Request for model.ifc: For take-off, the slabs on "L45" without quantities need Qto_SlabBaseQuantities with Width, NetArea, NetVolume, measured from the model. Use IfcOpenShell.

First a look at what the model holds.

```python
import ifcopenshell
import ifcopenshell.util.element
import ifcopenshell.util.unit

model = ifcopenshell.open("model.ifc")
print(model.schema)
for unit_type in ("LENGTHUNIT", "AREAUNIT", "VOLUMEUNIT"):
    print(unit_type, ifcopenshell.util.unit.calculate_unit_scale(model, unit_type))
storey = next(s for s in model.by_type("IfcBuildingStorey") if s.Name == "L45")
slabs = [e for e in ifcopenshell.util.element.get_decomposition(storey) if e.is_a("IfcSlab")]
for e in sorted(slabs, key=lambda e: e.id()):
    print(e.id(), e.is_a(), e.Name, list(ifcopenshell.util.element.get_psets(e, qtos_only=True)), sep=" | ")
```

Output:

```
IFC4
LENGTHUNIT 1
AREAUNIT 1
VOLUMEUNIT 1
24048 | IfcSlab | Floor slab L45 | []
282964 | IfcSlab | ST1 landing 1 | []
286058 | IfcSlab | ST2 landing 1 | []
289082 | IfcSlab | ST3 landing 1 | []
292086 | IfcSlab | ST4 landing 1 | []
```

```python
import ifcopenshell
import ifcopenshell.api.pset
import ifcopenshell.geom
import ifcopenshell.util.element
import ifcopenshell.util.shape
import ifcopenshell.util.unit

model = ifcopenshell.open("model.ifc")
unit_scale = ifcopenshell.util.unit.calculate_unit_scale(model)
area_scale = ifcopenshell.util.unit.calculate_unit_scale(model, "AREAUNIT")
volume_scale = ifcopenshell.util.unit.calculate_unit_scale(model, "VOLUMEUNIT")
settings = ifcopenshell.geom.settings()

storey = next(s for s in model.by_type("IfcBuildingStorey") if s.Name == "L45")
slabs = [e for e in ifcopenshell.util.element.get_decomposition(storey) if e.is_a("IfcSlab")]

for e in sorted(slabs, key=lambda e: e.id()):
    if ifcopenshell.util.element.get_psets(e, qtos_only=True, should_inherit=False):
        continue
    # Geometry comes back in metres, in the element's own axes.
    shape = ifcopenshell.geom.create_shape(settings, e)
    values = {
        "Width": ifcopenshell.util.shape.get_z(shape.geometry) / unit_scale,
        "NetArea": ifcopenshell.util.shape.get_footprint_area(shape.geometry) / area_scale,
        "NetVolume": ifcopenshell.util.shape.get_volume(shape.geometry) / volume_scale,
    }
    qto = ifcopenshell.api.pset.add_qto(model, product=e, name="Qto_SlabBaseQuantities")
    ifcopenshell.api.pset.edit_qto(model, qto=qto, properties=values)
    print(e.id(), {k: round(v, 3) for k, v in values.items()})

model.write("model_edited.ifc")
```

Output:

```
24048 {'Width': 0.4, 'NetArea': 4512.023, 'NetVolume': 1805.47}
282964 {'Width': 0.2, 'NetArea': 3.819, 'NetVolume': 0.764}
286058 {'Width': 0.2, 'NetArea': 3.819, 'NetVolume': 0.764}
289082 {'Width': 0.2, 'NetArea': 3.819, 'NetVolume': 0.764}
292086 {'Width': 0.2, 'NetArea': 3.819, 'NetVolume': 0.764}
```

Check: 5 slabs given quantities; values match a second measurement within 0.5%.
